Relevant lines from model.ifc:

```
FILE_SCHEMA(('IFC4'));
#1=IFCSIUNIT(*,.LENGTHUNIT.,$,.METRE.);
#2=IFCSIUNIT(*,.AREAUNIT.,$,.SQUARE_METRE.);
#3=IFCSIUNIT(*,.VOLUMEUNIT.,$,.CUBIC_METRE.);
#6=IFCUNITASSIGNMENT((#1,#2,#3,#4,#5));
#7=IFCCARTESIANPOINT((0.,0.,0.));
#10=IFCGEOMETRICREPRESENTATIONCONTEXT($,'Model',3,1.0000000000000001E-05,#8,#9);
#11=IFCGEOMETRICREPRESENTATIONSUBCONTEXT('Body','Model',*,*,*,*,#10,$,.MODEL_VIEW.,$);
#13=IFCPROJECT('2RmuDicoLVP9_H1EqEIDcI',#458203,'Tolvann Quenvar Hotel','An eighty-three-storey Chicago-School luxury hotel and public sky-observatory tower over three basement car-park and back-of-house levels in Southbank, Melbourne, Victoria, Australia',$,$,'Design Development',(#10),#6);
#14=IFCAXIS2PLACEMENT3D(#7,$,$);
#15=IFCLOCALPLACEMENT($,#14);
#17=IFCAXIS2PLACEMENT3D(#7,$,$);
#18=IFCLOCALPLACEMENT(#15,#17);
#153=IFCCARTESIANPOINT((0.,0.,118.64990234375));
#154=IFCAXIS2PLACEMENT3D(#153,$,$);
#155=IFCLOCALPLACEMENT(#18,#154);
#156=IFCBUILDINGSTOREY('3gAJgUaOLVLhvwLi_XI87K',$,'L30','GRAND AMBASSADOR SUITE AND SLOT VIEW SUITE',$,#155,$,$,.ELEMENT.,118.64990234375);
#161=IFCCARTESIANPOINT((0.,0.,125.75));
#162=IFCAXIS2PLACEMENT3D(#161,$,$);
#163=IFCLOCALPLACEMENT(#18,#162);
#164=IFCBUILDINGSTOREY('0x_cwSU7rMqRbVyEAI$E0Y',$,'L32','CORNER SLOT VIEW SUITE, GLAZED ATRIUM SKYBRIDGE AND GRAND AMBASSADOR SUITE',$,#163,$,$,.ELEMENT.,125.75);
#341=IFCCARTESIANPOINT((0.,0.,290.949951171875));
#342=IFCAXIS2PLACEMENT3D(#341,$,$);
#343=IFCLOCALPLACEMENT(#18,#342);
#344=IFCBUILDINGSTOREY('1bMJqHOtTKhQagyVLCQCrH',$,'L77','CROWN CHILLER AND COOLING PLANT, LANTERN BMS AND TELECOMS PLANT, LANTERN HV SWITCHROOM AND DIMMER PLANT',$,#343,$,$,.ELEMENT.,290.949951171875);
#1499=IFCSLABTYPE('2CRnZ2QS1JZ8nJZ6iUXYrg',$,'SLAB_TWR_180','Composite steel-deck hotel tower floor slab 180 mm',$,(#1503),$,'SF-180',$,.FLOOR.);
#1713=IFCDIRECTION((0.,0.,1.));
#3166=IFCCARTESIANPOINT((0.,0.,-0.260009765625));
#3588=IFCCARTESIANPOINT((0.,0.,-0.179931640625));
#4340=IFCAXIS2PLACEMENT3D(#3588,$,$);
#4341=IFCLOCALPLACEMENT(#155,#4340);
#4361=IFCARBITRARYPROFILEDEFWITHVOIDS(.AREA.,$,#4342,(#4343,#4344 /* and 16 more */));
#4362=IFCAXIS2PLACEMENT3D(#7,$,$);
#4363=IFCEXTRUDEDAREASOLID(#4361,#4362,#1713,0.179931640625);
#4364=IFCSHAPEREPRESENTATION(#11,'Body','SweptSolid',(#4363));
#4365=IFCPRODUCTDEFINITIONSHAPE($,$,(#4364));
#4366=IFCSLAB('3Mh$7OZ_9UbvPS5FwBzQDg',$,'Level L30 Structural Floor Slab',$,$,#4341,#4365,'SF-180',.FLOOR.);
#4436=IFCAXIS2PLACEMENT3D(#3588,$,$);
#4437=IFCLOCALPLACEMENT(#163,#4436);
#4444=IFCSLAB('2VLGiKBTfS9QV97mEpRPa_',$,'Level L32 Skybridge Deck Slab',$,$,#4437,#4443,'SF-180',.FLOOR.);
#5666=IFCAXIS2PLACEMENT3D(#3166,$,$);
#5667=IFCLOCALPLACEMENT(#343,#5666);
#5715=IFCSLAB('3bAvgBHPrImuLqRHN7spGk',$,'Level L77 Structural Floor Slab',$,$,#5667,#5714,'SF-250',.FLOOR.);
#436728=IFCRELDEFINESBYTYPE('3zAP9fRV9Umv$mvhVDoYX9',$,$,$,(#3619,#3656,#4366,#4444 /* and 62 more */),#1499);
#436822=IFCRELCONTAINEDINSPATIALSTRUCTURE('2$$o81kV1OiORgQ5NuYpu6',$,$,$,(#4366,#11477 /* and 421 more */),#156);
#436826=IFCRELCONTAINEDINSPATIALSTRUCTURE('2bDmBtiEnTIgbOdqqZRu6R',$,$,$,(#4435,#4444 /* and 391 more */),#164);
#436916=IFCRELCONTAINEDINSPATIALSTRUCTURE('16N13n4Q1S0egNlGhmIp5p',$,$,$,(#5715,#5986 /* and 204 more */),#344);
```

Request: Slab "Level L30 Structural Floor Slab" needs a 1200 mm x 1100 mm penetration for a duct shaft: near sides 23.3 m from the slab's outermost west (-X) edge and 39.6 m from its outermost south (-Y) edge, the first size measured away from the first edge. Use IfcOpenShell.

```python
import numpy as np
import ifcopenshell
import ifcopenshell.api.feature
import ifcopenshell.api.geometry
import ifcopenshell.api.root
import ifcopenshell.geom
import ifcopenshell.util.placement
import ifcopenshell.util.representation
import ifcopenshell.util.shape
import ifcopenshell.util.unit

model = ifcopenshell.open("model.ifc")
unit_scale = ifcopenshell.util.unit.calculate_unit_scale(model)
settings = ifcopenshell.geom.settings()


def volume(element):
    """Net volume in cubic metres, openings subtracted."""
    shape = ifcopenshell.geom.create_shape(settings, element)
    return ifcopenshell.util.shape.get_volume(shape.geometry)


slab = model.by_id(4366)
before = volume(slab)

# Extent in the slab's own axes, in metres. The edges named are its -X and -Y sides.
slab_shape = ifcopenshell.geom.create_shape(settings, slab)
vertices = ifcopenshell.util.shape.get_vertices(slab_shape.geometry)
x_min, y_min, bottom = vertices.min(axis=0)
top = vertices[:, 2].max()

opening = ifcopenshell.api.root.create_entity(model, ifc_class="IfcOpeningElement", name="Duct shaft opening", predefined_type="OPENING")
context = ifcopenshell.util.representation.get_context(model, "Model", "Body", "MODEL_VIEW")
width, depth = 1.2, 1.1
outline = [(0.0, 0.0), (width, 0.0), (width, depth), (0.0, depth), (0.0, 0.0)]
# Overshoot both faces by 50 mm so the cut is clean.
shape = ifcopenshell.api.geometry.add_slab_representation(
    model, context=context, depth=top - bottom + 0.1, polyline=outline
)
ifcopenshell.api.geometry.assign_representation(model, product=opening, representation=shape)

matrix = ifcopenshell.util.placement.get_local_placement(slab.ObjectPlacement)
matrix[:, 3] = matrix @ np.append(np.array([x_min + 23.3, y_min + 39.6, bottom - 0.05]) / unit_scale, 1.0)
ifcopenshell.api.geometry.edit_object_placement(model, product=opening, matrix=matrix, is_si=False)
ifcopenshell.api.feature.add_feature(model, feature=opening, element=slab)

after = volume(slab)

print(f"slab volume {before:.3f} -> {after:.3f} m3")

model.write("model_edited.ifc")
```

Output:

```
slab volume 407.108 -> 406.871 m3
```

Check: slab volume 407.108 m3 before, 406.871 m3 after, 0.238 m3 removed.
